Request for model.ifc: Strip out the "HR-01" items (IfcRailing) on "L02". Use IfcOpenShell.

First a look at what the model holds.

```python
import ifcopenshell
import ifcopenshell.util.element

model = ifcopenshell.open("model.ifc")
print(model.schema)
storey = next(s for s in model.by_type("IfcBuildingStorey") if s.Name == "L02")
railings = [e for e in ifcopenshell.util.element.get_decomposition(storey) if e.is_a("IfcRailing")]
seen = {}
for e in railings:
    element_type = ifcopenshell.util.element.get_type(e)
    name = element_type.Name if element_type not in (None, e) else None
    seen[name] = seen.get(name, 0) + 1
for name, count in sorted(seen.items(), key=str):
    print(count, "x", name)
```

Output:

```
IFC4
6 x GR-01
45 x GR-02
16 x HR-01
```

```python
import ifcopenshell
import ifcopenshell.api.root
import ifcopenshell.util.element

model = ifcopenshell.open("model.ifc")

storey = next(s for s in model.by_type("IfcBuildingStorey") if s.Name == "L02")
railings = [e for e in ifcopenshell.util.element.get_decomposition(storey) if e.is_a("IfcRailing")]
targets = [e for e in railings if (t := ifcopenshell.util.element.get_type(e)) not in (None, e) and t.Name == "HR-01"]

for e in targets:
    ifcopenshell.api.root.remove_product(model, product=e)
print(len(targets), "removed")

model.write("model_edited.ifc")
```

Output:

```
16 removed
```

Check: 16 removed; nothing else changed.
